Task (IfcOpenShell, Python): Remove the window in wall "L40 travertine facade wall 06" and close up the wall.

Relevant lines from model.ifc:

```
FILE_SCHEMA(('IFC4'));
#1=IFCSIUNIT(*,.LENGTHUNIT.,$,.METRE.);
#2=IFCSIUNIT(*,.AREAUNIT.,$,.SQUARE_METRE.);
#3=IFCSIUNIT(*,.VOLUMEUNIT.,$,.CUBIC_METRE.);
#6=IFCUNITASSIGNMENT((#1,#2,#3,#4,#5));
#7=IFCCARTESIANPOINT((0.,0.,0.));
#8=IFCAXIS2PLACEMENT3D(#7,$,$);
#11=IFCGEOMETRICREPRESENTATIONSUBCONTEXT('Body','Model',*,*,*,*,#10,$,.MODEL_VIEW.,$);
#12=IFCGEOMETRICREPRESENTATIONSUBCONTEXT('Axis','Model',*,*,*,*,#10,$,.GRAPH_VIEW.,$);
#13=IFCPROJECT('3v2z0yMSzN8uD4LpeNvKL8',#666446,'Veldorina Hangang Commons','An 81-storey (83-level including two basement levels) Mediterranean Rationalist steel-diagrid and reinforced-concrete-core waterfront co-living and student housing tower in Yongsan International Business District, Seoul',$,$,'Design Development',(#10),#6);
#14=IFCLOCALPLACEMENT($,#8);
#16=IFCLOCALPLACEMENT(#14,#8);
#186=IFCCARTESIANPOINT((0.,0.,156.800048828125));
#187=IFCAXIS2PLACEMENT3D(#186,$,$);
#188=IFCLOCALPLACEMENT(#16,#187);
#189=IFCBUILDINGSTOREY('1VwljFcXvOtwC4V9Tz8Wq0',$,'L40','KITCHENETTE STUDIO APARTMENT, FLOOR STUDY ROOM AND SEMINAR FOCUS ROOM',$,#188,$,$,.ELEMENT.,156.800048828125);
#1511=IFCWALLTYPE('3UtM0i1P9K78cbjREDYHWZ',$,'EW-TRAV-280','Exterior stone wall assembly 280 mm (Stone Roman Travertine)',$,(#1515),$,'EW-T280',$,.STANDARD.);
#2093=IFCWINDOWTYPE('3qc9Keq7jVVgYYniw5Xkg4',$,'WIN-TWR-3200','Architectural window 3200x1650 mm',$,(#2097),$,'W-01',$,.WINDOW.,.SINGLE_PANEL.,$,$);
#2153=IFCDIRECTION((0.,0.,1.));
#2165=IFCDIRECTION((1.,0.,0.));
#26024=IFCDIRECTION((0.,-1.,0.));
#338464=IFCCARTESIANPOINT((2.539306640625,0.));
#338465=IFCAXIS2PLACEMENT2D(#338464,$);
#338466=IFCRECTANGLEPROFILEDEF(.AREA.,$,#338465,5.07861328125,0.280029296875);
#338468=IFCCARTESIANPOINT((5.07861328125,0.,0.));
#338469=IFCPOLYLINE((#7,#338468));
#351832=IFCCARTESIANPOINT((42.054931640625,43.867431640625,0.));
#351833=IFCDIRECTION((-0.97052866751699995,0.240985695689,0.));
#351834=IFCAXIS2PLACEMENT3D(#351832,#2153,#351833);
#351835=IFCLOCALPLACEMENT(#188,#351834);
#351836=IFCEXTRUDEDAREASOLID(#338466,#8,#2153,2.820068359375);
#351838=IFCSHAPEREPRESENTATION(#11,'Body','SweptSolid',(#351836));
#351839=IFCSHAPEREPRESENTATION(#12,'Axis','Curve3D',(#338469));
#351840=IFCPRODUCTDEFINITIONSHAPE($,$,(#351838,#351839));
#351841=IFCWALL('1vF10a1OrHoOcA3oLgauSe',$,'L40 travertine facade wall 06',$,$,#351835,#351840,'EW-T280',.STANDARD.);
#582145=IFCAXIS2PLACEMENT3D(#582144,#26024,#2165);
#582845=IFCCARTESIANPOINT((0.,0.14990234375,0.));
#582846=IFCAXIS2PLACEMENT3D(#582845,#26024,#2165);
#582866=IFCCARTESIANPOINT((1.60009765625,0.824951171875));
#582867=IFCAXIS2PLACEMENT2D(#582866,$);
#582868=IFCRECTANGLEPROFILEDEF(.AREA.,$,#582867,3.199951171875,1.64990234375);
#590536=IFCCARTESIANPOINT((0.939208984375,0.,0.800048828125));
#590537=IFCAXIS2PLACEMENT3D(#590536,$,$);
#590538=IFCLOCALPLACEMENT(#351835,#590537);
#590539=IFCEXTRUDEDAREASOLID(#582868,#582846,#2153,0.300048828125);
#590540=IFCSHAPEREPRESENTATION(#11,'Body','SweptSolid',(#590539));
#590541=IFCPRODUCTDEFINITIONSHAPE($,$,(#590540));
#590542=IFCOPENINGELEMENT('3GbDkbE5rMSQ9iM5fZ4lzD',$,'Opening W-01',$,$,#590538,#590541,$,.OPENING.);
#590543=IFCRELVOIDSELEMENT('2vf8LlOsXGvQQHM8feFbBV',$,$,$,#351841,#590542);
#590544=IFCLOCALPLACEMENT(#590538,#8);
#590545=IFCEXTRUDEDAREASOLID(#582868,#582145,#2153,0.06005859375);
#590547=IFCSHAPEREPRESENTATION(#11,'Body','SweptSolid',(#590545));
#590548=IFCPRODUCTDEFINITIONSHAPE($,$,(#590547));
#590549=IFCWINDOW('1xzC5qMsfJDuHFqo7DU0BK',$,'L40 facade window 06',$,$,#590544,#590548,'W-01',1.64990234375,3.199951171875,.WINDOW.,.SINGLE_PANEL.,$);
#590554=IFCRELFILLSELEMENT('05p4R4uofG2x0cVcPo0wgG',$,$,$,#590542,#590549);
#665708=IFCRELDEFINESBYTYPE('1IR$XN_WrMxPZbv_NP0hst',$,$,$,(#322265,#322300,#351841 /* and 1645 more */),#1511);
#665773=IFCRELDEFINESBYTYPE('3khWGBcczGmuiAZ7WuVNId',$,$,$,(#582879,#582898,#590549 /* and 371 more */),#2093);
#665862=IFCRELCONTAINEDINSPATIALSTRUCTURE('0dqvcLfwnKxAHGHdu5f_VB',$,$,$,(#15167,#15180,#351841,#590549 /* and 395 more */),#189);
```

```python
import ifcopenshell
import ifcopenshell.api.feature
import ifcopenshell.api.root
import ifcopenshell.geom
import ifcopenshell.util.shape

model = ifcopenshell.open("model.ifc")
settings = ifcopenshell.geom.settings()


def volume(element):
    """Net volume in cubic metres, openings subtracted."""
    shape = ifcopenshell.geom.create_shape(settings, element)
    return ifcopenshell.util.shape.get_volume(shape.geometry)


window = model.by_guid("1xzC5qMsfJDuHFqo7DU0BK")
opening = window.FillsVoids[0].RelatingOpeningElement
wall = opening.VoidsElements[0].RelatingBuildingElement
before = volume(wall)

ifcopenshell.api.root.remove_product(model, product=window)
ifcopenshell.api.feature.remove_feature(model, feature=opening)

after = volume(wall)

print(f"wall volume {before:.3f} -> {after:.3f} m3")

model.write("model_updated.ifc")
```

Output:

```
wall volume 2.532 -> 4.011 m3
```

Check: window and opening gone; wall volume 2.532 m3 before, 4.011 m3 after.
